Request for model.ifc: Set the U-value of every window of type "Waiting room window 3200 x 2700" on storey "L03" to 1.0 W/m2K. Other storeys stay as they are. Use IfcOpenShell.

First a look at what the model holds.

```python
import ifcopenshell
import ifcopenshell.util.element

model = ifcopenshell.open("model.ifc")
print(model.schema)
storey = next(s for s in model.by_type("IfcBuildingStorey") if s.Name == "L03")
windows = [e for e in ifcopenshell.util.element.get_decomposition(storey) if e.is_a("IfcWindow")]
seen = {}
for e in windows:
    element_type = ifcopenshell.util.element.get_type(e)
    key = (element_type.Name if element_type != e and element_type else None, ifcopenshell.util.element.get_pset(e, "Pset_WindowCommon", "ThermalTransmittance"))
    seen[key] = seen.get(key, 0) + 1
for (name, value), count in sorted(seen.items(), key=str):
    print(count, "x", name, "|", value)
```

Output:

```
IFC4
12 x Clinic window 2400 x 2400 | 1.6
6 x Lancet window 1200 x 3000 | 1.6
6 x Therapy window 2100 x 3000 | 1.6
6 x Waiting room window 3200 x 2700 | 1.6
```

```python
import ifcopenshell
import ifcopenshell.api.pset
import ifcopenshell.util.element

model = ifcopenshell.open("model.ifc")

storey = next(s for s in model.by_type("IfcBuildingStorey") if s.Name == "L03")
windows = [e for e in ifcopenshell.util.element.get_decomposition(storey) if e.is_a("IfcWindow")]

count = 0
for e in windows:
    element_type = ifcopenshell.util.element.get_type(e)
    if element_type in (None, e) or element_type.Name != "Waiting room window 3200 x 2700":
        continue
    # add_pset returns the element's existing set when there is one.
    pset = ifcopenshell.api.pset.add_pset(model, product=e, name="Pset_WindowCommon")
    ifcopenshell.api.pset.edit_pset(model, pset=pset, properties={"ThermalTransmittance": 1.0})
    count += 1

print(count, "windows updated")

model.write("model_v2.ifc")
```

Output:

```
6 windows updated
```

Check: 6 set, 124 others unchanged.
